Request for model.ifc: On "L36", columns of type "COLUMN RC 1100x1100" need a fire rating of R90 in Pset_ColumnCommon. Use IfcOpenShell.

First a look at what the model holds.

```python
import ifcopenshell
import ifcopenshell.util.element

model = ifcopenshell.open("model.ifc")
print(model.schema)
storey = next(s for s in model.by_type("IfcBuildingStorey") if s.Name == "L36")
columns = [e for e in ifcopenshell.util.element.get_decomposition(storey) if e.is_a("IfcColumn")]
seen = {}
for e in columns:
    element_type = ifcopenshell.util.element.get_type(e)
    key = (element_type.Name if element_type != e and element_type else None, ifcopenshell.util.element.get_pset(e, "Pset_ColumnCommon", "FireRating"))
    seen[key] = seen.get(key, 0) + 1
for (name, value), count in sorted(seen.items(), key=str):
    print(count, "x", name, "|", value)
```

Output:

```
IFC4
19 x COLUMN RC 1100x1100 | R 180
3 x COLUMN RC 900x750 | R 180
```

```python
import ifcopenshell
import ifcopenshell.api.pset
import ifcopenshell.util.element

model = ifcopenshell.open("model.ifc")

storey = next(s for s in model.by_type("IfcBuildingStorey") if s.Name == "L36")
columns = [e for e in ifcopenshell.util.element.get_decomposition(storey) if e.is_a("IfcColumn")]

count = 0
for e in columns:
    element_type = ifcopenshell.util.element.get_type(e)
    if element_type in (None, e) or element_type.Name != "COLUMN RC 1100x1100":
        continue
    found = ifcopenshell.util.element.get_pset(e, "Pset_ColumnCommon", should_inherit=False)
    if found:
        pset = model.by_id(found["id"])
        if len(ifcopenshell.util.element.get_elements_by_pset(pset)) > 1:
            pset = ifcopenshell.api.pset.unshare_pset(model, products=[e], pset=pset)[0]
    else:
        pset = ifcopenshell.api.pset.add_pset(model, product=e, name="Pset_ColumnCommon")
    ifcopenshell.api.pset.edit_pset(model, pset=pset, properties={"FireRating": "R90"})
    count += 1

print(count, "columns updated")

model.write("model_v2.ifc")
```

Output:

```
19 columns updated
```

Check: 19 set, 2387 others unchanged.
